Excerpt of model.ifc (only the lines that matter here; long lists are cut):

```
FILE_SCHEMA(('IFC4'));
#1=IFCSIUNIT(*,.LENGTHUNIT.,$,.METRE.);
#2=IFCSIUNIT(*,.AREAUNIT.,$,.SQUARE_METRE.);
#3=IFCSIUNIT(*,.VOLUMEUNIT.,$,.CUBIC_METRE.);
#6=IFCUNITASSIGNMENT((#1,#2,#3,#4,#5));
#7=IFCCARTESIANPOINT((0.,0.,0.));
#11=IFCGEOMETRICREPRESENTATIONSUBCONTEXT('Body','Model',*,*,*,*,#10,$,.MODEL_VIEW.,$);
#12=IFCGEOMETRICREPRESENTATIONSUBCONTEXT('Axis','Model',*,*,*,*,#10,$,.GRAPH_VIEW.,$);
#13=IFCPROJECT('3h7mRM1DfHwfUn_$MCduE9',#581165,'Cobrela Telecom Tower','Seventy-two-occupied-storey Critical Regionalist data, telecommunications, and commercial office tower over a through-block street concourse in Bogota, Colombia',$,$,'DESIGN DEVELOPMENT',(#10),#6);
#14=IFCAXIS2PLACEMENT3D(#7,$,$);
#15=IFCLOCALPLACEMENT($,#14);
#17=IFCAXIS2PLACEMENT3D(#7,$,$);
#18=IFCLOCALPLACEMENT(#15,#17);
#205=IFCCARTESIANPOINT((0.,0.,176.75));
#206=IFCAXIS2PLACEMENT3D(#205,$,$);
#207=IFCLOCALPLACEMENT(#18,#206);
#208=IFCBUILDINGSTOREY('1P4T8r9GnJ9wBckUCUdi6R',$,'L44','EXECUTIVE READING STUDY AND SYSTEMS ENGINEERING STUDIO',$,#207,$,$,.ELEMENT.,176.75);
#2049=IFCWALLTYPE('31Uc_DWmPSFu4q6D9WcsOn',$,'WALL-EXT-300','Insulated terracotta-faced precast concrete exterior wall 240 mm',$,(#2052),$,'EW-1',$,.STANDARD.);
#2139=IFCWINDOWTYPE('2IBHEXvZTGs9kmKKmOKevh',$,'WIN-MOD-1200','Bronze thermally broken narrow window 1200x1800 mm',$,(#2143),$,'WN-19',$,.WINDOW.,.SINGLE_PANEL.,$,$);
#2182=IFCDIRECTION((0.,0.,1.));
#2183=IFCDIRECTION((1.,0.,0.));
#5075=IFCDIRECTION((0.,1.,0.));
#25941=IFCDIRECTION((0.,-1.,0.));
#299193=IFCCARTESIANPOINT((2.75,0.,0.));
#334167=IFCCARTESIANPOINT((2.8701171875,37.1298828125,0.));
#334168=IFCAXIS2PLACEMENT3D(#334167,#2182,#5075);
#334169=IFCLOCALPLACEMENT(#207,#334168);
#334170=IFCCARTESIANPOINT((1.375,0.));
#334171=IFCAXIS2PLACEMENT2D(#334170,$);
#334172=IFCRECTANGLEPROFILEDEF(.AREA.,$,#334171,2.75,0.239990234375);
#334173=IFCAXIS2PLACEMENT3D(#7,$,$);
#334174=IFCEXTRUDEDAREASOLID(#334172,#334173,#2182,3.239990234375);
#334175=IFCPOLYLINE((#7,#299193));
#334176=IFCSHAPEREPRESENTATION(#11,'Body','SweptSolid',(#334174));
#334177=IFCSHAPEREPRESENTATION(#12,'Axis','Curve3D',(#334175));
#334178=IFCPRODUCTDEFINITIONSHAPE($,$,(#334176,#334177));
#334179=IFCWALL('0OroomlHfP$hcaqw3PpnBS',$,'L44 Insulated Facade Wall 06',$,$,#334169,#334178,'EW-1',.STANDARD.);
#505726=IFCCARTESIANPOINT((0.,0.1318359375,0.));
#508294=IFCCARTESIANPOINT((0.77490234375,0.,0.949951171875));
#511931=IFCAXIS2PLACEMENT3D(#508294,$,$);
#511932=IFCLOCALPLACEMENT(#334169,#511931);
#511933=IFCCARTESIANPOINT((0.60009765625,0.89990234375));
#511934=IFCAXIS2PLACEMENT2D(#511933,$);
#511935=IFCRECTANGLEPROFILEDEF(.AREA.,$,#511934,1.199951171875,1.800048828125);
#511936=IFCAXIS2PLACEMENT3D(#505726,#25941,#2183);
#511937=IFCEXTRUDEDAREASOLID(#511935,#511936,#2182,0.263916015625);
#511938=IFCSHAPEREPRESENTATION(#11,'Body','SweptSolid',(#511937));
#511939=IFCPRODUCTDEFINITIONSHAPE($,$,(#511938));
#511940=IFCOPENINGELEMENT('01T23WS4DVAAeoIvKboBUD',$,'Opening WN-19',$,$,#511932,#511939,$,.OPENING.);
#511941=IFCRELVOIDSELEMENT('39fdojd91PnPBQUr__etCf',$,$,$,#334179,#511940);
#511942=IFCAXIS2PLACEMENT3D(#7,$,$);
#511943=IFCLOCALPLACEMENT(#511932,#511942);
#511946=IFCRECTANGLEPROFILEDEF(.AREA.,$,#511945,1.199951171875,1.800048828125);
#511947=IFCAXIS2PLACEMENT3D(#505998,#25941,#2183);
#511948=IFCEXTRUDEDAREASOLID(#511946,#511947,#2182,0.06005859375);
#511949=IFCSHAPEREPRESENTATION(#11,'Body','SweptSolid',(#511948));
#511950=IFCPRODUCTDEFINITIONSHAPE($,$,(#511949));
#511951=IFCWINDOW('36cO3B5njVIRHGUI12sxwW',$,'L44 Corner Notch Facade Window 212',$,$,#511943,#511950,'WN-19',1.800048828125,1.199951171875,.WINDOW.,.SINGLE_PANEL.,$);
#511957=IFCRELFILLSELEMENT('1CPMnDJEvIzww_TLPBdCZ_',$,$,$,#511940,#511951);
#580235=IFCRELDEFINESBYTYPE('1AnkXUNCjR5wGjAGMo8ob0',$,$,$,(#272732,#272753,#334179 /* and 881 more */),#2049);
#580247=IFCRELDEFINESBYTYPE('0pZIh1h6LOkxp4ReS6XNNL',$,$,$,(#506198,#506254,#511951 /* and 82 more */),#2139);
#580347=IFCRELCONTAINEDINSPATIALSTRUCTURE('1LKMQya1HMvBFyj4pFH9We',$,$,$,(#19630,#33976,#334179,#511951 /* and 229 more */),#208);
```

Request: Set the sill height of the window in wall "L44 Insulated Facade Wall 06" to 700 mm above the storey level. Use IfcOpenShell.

```python
import numpy as np
import ifcopenshell
import ifcopenshell.api.geometry
import ifcopenshell.geom
import ifcopenshell.util.element
import ifcopenshell.util.placement
import ifcopenshell.util.shape
import ifcopenshell.util.unit

model = ifcopenshell.open("model.ifc")
unit_scale = ifcopenshell.util.unit.calculate_unit_scale(model)

window = model.by_id(511951)
opening = window.FillsVoids[0].RelatingOpeningElement
storey = ifcopenshell.util.element.get_container(window, ifc_class="IfcBuildingStorey")
level = ifcopenshell.util.placement.get_local_placement(storey.ObjectPlacement)[2, 3]

# The opening's origin need not be at the sill, so measure its lowest point.
shape = ifcopenshell.geom.create_shape(ifcopenshell.geom.settings(), opening)
bottom = ifcopenshell.util.shape.get_shape_bottom_elevation(shape, shape.geometry) / unit_scale
dz = level + 0.7 / unit_scale - bottom

shift = np.array([0.0, 0.0, dz])
# The window is placed relative to its opening, so it follows when the opening moves.
matrix = ifcopenshell.util.placement.get_local_placement(opening.ObjectPlacement)
matrix[:3, 3] += shift
ifcopenshell.api.geometry.edit_object_placement(
    model, product=opening, matrix=matrix, is_si=False, should_transform_children=True
)

print(f"moved by {dz * unit_scale:+.3f} m")

model.write("model_v2.ifc")
```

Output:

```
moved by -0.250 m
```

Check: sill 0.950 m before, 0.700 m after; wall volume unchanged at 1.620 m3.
